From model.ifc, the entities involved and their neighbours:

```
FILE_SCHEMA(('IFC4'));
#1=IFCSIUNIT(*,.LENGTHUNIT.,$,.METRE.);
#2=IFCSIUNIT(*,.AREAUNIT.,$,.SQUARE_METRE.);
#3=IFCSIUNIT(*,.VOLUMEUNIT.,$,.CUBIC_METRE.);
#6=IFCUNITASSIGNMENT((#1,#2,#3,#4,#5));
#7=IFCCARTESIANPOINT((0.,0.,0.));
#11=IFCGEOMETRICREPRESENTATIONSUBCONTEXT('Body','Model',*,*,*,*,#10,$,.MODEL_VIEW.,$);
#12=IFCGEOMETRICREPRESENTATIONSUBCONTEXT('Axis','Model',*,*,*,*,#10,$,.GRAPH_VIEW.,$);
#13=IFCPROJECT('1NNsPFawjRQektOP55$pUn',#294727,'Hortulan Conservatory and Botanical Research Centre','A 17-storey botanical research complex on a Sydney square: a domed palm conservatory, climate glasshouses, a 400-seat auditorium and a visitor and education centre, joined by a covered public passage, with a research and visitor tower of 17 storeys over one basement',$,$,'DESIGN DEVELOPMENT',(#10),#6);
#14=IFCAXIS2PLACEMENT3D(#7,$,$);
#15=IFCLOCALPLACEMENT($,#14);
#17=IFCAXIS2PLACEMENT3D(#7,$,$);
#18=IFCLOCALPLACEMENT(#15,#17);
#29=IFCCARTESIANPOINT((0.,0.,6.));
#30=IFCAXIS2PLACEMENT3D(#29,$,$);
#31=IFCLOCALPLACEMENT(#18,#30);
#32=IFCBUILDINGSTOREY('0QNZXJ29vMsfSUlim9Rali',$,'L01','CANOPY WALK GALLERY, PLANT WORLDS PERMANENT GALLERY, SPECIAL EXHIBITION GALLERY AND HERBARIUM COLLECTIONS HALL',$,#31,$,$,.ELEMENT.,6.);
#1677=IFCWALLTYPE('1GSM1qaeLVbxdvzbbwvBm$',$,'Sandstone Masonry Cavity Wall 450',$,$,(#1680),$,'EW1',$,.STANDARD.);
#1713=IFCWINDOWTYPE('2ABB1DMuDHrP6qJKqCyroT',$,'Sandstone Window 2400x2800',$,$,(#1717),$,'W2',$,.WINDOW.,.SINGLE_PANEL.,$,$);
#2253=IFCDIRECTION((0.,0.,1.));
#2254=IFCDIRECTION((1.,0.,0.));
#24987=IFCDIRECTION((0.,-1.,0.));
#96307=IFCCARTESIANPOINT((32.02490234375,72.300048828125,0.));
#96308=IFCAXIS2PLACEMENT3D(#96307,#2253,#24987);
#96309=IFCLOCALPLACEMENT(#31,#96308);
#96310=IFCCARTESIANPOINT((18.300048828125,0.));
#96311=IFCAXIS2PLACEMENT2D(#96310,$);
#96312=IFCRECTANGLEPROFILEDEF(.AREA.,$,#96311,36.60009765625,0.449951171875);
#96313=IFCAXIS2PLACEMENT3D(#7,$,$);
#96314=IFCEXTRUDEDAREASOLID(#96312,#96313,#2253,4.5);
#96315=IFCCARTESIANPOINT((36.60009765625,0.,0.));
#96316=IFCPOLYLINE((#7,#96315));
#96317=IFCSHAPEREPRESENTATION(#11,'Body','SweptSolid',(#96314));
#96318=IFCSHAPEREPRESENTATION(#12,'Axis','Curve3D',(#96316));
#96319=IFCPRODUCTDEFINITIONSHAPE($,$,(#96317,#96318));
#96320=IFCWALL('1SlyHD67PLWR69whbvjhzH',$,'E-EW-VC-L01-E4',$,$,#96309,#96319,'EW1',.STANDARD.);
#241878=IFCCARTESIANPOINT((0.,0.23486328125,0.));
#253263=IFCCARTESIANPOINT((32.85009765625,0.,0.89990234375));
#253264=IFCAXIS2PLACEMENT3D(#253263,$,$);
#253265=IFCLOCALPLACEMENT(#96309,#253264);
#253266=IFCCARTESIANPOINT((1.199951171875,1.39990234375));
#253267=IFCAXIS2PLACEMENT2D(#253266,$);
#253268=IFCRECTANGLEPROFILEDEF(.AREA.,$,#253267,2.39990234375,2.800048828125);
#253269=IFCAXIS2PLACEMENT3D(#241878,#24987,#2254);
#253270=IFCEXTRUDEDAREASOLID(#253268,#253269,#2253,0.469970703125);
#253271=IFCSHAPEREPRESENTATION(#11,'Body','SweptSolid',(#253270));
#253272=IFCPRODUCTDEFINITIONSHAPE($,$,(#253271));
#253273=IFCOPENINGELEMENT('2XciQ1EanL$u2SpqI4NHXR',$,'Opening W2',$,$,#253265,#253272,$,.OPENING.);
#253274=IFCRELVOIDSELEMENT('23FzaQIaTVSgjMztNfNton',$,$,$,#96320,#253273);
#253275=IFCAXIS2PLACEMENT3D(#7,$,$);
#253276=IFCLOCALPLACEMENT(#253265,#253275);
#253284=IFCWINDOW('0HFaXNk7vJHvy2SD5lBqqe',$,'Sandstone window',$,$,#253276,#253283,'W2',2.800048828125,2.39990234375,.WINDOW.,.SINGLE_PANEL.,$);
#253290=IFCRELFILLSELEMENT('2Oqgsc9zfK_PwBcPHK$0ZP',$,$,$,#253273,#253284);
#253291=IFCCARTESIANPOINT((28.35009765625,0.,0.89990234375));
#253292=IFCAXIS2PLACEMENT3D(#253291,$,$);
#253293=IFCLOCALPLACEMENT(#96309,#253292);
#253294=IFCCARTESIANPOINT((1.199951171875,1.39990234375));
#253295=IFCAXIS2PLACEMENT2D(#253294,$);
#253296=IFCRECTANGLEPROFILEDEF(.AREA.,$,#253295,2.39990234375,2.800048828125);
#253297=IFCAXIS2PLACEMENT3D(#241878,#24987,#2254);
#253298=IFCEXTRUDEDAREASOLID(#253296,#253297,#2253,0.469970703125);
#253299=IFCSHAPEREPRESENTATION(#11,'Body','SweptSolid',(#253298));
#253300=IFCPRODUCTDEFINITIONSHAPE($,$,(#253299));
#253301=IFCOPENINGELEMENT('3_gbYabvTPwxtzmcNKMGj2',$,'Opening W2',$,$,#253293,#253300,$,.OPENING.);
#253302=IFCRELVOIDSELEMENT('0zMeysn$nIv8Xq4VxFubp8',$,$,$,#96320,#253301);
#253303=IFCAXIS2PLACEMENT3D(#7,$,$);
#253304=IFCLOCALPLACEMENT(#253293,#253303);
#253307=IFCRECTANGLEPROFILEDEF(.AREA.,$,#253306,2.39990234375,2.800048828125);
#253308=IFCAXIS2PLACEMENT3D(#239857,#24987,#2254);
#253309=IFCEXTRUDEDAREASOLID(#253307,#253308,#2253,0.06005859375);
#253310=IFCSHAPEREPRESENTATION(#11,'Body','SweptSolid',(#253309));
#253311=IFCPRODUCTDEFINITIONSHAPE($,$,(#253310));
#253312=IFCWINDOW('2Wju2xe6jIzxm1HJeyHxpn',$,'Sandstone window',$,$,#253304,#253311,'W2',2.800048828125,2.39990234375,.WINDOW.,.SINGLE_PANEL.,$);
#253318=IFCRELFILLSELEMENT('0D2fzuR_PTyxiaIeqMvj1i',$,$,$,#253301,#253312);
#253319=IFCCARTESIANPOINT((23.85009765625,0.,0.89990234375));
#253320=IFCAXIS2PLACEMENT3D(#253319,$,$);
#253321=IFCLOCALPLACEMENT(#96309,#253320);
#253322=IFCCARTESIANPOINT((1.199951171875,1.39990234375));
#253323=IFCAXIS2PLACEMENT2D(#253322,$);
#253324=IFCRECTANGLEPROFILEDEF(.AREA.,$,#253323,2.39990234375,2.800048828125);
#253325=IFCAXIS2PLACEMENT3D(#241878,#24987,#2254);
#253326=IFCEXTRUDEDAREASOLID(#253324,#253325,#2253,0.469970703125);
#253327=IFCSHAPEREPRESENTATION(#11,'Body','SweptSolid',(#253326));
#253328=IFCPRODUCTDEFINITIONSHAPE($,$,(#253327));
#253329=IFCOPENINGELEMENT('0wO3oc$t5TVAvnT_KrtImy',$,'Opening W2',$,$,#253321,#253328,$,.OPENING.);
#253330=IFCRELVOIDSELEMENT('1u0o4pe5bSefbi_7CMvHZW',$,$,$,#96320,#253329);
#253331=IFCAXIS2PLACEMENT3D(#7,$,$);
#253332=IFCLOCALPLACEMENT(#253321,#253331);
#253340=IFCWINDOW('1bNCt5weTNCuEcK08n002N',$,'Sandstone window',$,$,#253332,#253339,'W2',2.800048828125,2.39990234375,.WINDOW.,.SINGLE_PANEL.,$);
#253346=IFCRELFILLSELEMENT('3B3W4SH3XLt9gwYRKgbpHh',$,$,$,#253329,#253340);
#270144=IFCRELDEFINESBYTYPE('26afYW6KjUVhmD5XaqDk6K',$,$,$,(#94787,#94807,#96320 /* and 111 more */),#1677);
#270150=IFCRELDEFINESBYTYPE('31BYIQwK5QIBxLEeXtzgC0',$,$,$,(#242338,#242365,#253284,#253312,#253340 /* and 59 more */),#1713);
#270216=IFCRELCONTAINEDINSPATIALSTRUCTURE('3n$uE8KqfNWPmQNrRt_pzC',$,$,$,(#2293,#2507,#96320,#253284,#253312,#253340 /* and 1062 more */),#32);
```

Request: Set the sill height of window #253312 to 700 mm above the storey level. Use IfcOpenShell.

```python
import numpy as np
import ifcopenshell
import ifcopenshell.api.geometry
import ifcopenshell.geom
import ifcopenshell.util.element
import ifcopenshell.util.placement
import ifcopenshell.util.shape
import ifcopenshell.util.unit

model = ifcopenshell.open("model.ifc")
unit_scale = ifcopenshell.util.unit.calculate_unit_scale(model)

window = model.by_guid("2Wju2xe6jIzxm1HJeyHxpn")
opening = window.FillsVoids[0].RelatingOpeningElement
storey = ifcopenshell.util.element.get_container(window, ifc_class="IfcBuildingStorey")
level = ifcopenshell.util.placement.get_local_placement(storey.ObjectPlacement)[2, 3]

# The opening's origin need not be at the sill, so measure its lowest point.
shape = ifcopenshell.geom.create_shape(ifcopenshell.geom.settings(), opening)
bottom = ifcopenshell.util.shape.get_shape_bottom_elevation(shape, shape.geometry) / unit_scale
dz = level + 0.7 - bottom

shift = np.array([0.0, 0.0, dz])
# The window is placed relative to its opening, so it follows when the opening moves.
matrix = ifcopenshell.util.placement.get_local_placement(opening.ObjectPlacement)
matrix[:3, 3] += shift
ifcopenshell.api.geometry.edit_object_placement(
    model, product=opening, matrix=matrix, is_si=False, should_transform_children=True
)

print(f"moved by {dz * unit_scale:+.3f} m")

model.write("model_updated.ifc")
```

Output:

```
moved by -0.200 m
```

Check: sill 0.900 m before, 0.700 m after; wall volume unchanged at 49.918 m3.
